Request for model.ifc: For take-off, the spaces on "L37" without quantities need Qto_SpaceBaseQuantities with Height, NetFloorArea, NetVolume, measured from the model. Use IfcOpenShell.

First a look at what the model holds.

```python
import ifcopenshell
import ifcopenshell.util.element
import ifcopenshell.util.unit

model = ifcopenshell.open("model.ifc")
print(model.schema)
for unit_type in ("LENGTHUNIT", "AREAUNIT", "VOLUMEUNIT"):
    print(unit_type, ifcopenshell.util.unit.calculate_unit_scale(model, unit_type))
storey = next(s for s in model.by_type("IfcBuildingStorey") if s.Name == "L37")
spaces = [e for e in ifcopenshell.util.element.get_decomposition(storey) if e.is_a("IfcSpace")]
for e in sorted(spaces, key=lambda e: e.id()):
    print(e.id(), e.is_a(), e.Name, list(ifcopenshell.util.element.get_psets(e, qtos_only=True)), sep=" | ")
```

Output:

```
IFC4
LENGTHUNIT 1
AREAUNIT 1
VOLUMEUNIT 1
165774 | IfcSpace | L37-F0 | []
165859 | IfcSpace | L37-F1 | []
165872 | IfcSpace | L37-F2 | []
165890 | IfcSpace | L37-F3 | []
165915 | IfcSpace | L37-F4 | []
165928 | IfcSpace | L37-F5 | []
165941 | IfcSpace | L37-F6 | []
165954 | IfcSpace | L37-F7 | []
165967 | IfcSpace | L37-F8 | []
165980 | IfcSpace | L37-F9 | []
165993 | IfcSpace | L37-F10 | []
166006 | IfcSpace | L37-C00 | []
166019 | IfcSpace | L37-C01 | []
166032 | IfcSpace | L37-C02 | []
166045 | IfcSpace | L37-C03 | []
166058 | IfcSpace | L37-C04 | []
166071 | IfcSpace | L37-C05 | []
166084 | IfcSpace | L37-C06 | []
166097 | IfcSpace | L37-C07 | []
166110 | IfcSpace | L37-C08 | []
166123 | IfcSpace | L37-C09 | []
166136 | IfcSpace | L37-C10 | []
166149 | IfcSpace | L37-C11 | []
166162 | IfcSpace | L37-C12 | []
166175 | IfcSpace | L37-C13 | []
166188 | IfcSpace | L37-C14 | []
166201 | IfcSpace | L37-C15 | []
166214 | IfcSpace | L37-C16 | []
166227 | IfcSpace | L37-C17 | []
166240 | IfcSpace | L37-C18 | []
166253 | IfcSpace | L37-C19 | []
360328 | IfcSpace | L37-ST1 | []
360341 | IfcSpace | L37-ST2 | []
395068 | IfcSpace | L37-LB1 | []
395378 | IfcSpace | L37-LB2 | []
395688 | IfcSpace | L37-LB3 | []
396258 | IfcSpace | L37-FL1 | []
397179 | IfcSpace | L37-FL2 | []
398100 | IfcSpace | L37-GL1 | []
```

```python
import ifcopenshell
import ifcopenshell.api.pset
import ifcopenshell.geom
import ifcopenshell.util.element
import ifcopenshell.util.shape
import ifcopenshell.util.unit

model = ifcopenshell.open("model.ifc")
unit_scale = ifcopenshell.util.unit.calculate_unit_scale(model)
area_scale = ifcopenshell.util.unit.calculate_unit_scale(model, "AREAUNIT")
volume_scale = ifcopenshell.util.unit.calculate_unit_scale(model, "VOLUMEUNIT")
settings = ifcopenshell.geom.settings()

storey = next(s for s in model.by_type("IfcBuildingStorey") if s.Name == "L37")
spaces = [e for e in ifcopenshell.util.element.get_decomposition(storey) if e.is_a("IfcSpace")]

for e in sorted(spaces, key=lambda e: e.id()):
    if ifcopenshell.util.element.get_psets(e, qtos_only=True, should_inherit=False):
        continue
    # Geometry comes back in metres, in the element's own axes.
    shape = ifcopenshell.geom.create_shape(settings, e)
    values = {
        "Height": ifcopenshell.util.shape.get_z(shape.geometry) / unit_scale,
        "NetFloorArea": ifcopenshell.util.shape.get_footprint_area(shape.geometry) / area_scale,
        "NetVolume": ifcopenshell.util.shape.get_volume(shape.geometry) / volume_scale,
    }
    qto = ifcopenshell.api.pset.add_qto(model, product=e, name="Qto_SpaceBaseQuantities")
    ifcopenshell.api.pset.edit_qto(model, qto=qto, properties=values)
    print(e.id(), {k: round(v, 3) for k, v in values.items()})

model.write("model_v2.ifc")
```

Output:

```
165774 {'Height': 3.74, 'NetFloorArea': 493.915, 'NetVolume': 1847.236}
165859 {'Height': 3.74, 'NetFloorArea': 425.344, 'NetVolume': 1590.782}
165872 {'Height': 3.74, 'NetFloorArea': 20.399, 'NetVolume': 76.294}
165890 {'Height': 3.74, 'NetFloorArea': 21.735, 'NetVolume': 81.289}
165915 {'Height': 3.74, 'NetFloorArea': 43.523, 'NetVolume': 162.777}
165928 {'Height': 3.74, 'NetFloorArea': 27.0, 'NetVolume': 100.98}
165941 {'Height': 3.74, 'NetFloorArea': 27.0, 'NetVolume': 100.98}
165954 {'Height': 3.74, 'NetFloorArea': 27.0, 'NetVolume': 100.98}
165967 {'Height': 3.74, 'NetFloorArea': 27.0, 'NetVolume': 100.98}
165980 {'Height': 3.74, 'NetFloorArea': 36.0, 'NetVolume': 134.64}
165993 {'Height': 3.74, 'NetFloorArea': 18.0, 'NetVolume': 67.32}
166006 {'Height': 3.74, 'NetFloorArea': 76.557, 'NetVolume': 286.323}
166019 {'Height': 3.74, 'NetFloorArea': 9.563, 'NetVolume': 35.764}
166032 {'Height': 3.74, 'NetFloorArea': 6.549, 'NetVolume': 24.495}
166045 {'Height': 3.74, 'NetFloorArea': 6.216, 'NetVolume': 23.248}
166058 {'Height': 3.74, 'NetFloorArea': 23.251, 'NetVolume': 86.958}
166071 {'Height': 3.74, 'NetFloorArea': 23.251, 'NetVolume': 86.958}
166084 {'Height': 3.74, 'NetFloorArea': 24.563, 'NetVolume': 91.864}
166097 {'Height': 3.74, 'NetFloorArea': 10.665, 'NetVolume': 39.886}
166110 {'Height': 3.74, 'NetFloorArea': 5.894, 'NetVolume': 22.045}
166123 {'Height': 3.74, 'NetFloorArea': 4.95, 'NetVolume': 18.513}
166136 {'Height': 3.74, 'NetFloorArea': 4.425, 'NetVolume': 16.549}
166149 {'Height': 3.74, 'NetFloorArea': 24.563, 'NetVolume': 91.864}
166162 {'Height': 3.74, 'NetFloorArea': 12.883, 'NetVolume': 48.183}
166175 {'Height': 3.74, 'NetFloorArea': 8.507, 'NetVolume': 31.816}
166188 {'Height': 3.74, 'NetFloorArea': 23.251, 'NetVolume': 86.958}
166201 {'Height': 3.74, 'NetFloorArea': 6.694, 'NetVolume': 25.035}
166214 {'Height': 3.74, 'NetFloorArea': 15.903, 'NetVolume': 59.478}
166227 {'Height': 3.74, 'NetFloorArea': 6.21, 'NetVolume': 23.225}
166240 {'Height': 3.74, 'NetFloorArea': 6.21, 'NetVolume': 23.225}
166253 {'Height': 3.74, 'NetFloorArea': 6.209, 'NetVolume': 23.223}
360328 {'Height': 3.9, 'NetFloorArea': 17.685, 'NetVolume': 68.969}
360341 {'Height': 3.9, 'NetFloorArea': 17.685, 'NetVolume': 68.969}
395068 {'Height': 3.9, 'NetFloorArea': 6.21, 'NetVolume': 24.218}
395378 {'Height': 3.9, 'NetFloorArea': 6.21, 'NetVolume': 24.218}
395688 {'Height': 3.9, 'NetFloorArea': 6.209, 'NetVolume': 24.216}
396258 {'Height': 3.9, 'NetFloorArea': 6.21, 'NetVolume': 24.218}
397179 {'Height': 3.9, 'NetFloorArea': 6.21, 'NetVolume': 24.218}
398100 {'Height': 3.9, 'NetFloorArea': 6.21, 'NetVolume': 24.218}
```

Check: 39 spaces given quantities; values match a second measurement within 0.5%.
